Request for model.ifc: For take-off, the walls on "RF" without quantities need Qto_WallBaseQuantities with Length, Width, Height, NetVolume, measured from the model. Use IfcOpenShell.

First a look at what the model holds.

```python
import ifcopenshell
import ifcopenshell.util.element
import ifcopenshell.util.unit

model = ifcopenshell.open("model.ifc")
print(model.schema)
for unit_type in ("LENGTHUNIT", "AREAUNIT", "VOLUMEUNIT"):
    print(unit_type, ifcopenshell.util.unit.calculate_unit_scale(model, unit_type))
storey = next(s for s in model.by_type("IfcBuildingStorey") if s.Name == "RF")
walls = [e for e in ifcopenshell.util.element.get_decomposition(storey) if e.is_a("IfcWall")]
for e in sorted(walls, key=lambda e: e.id()):
    print(e.id(), e.is_a(), e.Name, list(ifcopenshell.util.element.get_psets(e, qtos_only=True)), sep=" | ")
```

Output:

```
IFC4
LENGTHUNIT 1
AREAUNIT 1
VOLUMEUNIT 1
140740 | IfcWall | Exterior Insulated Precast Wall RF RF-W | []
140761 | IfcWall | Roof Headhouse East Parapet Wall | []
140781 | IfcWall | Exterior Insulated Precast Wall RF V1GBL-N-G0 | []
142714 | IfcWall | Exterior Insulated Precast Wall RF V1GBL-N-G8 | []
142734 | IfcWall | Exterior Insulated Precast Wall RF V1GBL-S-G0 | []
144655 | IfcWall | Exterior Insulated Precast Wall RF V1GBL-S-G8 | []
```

```python
import ifcopenshell
import ifcopenshell.api.pset
import ifcopenshell.geom
import ifcopenshell.util.element
import ifcopenshell.util.shape
import ifcopenshell.util.unit

model = ifcopenshell.open("model.ifc")
unit_scale = ifcopenshell.util.unit.calculate_unit_scale(model)
volume_scale = ifcopenshell.util.unit.calculate_unit_scale(model, "VOLUMEUNIT")
settings = ifcopenshell.geom.settings()

storey = next(s for s in model.by_type("IfcBuildingStorey") if s.Name == "RF")
walls = [e for e in ifcopenshell.util.element.get_decomposition(storey) if e.is_a("IfcWall")]

for e in sorted(walls, key=lambda e: e.id()):
    if ifcopenshell.util.element.get_psets(e, qtos_only=True, should_inherit=False):
        continue
    # Geometry comes back in metres, in the element's own axes.
    shape = ifcopenshell.geom.create_shape(settings, e)
    values = {
        "Length": ifcopenshell.util.shape.get_x(shape.geometry) / unit_scale,
        "Width": ifcopenshell.util.shape.get_y(shape.geometry) / unit_scale,
        "Height": ifcopenshell.util.shape.get_z(shape.geometry) / unit_scale,
        "NetVolume": ifcopenshell.util.shape.get_volume(shape.geometry) / volume_scale,
    }
    qto = ifcopenshell.api.pset.add_qto(model, product=e, name="Qto_WallBaseQuantities")
    ifcopenshell.api.pset.edit_qto(model, qto=qto, properties=values)
    print(e.id(), {k: round(v, 3) for k, v in values.items()})

model.write("model_updated.ifc")
```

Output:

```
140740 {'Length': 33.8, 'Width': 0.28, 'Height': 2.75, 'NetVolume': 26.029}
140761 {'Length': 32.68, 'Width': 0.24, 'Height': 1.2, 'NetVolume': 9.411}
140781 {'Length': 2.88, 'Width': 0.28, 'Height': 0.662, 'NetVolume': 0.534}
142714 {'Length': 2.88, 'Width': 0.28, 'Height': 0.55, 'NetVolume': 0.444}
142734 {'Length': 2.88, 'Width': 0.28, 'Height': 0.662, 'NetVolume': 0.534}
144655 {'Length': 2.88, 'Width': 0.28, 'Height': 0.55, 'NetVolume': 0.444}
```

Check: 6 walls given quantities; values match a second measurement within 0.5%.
